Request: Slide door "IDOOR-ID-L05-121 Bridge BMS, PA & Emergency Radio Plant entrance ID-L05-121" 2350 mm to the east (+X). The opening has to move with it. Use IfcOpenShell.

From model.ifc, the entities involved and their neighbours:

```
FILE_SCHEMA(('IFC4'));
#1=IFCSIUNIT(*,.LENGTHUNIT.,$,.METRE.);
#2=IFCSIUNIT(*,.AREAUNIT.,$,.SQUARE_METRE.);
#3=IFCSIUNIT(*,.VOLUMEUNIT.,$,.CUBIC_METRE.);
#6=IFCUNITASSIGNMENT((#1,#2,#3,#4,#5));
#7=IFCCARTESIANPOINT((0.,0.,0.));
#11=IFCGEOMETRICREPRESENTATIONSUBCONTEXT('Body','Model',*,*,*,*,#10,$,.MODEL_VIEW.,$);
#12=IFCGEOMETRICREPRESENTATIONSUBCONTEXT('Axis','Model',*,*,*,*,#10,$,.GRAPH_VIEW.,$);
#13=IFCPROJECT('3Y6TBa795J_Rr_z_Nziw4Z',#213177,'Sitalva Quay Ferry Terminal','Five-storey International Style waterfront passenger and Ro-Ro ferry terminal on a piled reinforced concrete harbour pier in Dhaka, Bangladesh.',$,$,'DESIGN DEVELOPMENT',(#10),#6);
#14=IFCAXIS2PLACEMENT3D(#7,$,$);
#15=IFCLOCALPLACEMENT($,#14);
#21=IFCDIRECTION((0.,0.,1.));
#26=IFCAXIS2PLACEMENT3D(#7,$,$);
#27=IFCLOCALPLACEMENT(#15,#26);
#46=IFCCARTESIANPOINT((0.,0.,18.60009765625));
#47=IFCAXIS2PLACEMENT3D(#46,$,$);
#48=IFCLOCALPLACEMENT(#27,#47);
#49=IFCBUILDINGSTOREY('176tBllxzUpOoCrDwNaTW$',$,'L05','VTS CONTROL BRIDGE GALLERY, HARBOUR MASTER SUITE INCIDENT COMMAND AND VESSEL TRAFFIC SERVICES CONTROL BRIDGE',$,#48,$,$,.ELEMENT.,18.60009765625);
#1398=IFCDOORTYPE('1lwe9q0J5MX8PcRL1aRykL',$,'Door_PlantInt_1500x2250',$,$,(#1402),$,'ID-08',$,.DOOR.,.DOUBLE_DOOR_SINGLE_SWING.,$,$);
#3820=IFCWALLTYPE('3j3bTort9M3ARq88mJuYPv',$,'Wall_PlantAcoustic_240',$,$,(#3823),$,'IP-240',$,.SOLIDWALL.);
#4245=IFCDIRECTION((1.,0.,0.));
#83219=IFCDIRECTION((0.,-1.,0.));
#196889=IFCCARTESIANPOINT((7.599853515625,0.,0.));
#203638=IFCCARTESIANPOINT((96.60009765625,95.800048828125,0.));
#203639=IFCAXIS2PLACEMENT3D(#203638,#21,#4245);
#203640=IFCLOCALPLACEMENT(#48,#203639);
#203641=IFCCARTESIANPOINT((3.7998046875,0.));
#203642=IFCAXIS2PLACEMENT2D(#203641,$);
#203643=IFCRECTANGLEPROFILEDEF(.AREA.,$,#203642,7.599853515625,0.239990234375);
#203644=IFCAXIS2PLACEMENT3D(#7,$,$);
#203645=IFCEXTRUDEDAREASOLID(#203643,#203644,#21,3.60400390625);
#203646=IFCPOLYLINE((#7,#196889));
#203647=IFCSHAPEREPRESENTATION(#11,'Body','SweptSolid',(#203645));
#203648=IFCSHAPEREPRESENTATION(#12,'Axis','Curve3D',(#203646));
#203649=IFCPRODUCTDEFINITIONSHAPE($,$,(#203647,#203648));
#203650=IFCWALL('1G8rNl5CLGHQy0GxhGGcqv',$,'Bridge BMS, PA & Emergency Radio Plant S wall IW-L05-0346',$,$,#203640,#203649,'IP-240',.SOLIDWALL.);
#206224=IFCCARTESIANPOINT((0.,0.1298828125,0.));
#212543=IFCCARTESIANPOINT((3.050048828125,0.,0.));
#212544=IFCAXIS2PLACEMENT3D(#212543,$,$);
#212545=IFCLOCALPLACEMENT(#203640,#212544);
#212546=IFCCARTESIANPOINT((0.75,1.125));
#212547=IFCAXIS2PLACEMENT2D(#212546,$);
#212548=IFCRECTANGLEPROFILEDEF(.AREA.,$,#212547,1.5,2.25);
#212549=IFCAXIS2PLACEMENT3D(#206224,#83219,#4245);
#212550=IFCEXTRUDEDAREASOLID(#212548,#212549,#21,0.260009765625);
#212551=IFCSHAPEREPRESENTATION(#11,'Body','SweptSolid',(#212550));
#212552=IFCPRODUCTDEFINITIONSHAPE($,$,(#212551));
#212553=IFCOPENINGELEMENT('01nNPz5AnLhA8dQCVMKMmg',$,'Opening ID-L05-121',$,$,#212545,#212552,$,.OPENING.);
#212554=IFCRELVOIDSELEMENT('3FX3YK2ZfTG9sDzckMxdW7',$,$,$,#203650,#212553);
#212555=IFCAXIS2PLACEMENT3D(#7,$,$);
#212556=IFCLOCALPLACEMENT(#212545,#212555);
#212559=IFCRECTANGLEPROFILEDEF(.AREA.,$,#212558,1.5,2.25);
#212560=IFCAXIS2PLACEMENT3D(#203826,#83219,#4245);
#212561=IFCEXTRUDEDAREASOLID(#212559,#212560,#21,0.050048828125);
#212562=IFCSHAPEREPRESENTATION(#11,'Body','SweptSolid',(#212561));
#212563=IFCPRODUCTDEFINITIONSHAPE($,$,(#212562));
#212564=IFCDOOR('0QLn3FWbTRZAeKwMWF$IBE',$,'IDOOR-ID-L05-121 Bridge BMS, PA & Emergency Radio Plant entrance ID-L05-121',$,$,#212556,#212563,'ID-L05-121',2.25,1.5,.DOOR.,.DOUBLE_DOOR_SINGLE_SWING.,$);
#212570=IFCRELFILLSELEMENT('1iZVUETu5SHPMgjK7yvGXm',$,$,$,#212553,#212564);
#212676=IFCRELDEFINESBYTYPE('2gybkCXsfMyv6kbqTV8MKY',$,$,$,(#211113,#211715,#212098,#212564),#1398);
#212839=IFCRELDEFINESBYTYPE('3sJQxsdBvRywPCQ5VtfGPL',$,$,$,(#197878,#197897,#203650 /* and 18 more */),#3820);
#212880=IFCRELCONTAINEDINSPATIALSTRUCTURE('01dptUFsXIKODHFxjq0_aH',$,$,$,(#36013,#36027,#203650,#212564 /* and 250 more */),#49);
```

```python
import ifcopenshell
import ifcopenshell.api.geometry
import ifcopenshell.util.placement

model = ifcopenshell.open("model.ifc")

door = model.by_id(212564)
opening = door.FillsVoids[0].RelatingOpeningElement
wall = opening.VoidsElements[0].RelatingBuildingElement

wall_matrix = ifcopenshell.util.placement.get_local_placement(wall.ObjectPlacement)
shift = wall_matrix[:3, 0] * 2.35
before = ifcopenshell.util.placement.get_local_placement(door.ObjectPlacement)[:3, 3].copy()

# The door is placed relative to its opening, so it follows when the opening moves.
matrix = ifcopenshell.util.placement.get_local_placement(opening.ObjectPlacement)
matrix[:3, 3] += shift
ifcopenshell.api.geometry.edit_object_placement(
    model, product=opening, matrix=matrix, is_si=False, should_transform_children=True
)

after = ifcopenshell.util.placement.get_local_placement(door.ObjectPlacement)[:3, 3]
print("door moved by", (after - before).round(3) + 0.0)

model.write("model_v2.ifc")
```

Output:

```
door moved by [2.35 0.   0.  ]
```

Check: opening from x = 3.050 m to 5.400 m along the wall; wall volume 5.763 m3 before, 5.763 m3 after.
